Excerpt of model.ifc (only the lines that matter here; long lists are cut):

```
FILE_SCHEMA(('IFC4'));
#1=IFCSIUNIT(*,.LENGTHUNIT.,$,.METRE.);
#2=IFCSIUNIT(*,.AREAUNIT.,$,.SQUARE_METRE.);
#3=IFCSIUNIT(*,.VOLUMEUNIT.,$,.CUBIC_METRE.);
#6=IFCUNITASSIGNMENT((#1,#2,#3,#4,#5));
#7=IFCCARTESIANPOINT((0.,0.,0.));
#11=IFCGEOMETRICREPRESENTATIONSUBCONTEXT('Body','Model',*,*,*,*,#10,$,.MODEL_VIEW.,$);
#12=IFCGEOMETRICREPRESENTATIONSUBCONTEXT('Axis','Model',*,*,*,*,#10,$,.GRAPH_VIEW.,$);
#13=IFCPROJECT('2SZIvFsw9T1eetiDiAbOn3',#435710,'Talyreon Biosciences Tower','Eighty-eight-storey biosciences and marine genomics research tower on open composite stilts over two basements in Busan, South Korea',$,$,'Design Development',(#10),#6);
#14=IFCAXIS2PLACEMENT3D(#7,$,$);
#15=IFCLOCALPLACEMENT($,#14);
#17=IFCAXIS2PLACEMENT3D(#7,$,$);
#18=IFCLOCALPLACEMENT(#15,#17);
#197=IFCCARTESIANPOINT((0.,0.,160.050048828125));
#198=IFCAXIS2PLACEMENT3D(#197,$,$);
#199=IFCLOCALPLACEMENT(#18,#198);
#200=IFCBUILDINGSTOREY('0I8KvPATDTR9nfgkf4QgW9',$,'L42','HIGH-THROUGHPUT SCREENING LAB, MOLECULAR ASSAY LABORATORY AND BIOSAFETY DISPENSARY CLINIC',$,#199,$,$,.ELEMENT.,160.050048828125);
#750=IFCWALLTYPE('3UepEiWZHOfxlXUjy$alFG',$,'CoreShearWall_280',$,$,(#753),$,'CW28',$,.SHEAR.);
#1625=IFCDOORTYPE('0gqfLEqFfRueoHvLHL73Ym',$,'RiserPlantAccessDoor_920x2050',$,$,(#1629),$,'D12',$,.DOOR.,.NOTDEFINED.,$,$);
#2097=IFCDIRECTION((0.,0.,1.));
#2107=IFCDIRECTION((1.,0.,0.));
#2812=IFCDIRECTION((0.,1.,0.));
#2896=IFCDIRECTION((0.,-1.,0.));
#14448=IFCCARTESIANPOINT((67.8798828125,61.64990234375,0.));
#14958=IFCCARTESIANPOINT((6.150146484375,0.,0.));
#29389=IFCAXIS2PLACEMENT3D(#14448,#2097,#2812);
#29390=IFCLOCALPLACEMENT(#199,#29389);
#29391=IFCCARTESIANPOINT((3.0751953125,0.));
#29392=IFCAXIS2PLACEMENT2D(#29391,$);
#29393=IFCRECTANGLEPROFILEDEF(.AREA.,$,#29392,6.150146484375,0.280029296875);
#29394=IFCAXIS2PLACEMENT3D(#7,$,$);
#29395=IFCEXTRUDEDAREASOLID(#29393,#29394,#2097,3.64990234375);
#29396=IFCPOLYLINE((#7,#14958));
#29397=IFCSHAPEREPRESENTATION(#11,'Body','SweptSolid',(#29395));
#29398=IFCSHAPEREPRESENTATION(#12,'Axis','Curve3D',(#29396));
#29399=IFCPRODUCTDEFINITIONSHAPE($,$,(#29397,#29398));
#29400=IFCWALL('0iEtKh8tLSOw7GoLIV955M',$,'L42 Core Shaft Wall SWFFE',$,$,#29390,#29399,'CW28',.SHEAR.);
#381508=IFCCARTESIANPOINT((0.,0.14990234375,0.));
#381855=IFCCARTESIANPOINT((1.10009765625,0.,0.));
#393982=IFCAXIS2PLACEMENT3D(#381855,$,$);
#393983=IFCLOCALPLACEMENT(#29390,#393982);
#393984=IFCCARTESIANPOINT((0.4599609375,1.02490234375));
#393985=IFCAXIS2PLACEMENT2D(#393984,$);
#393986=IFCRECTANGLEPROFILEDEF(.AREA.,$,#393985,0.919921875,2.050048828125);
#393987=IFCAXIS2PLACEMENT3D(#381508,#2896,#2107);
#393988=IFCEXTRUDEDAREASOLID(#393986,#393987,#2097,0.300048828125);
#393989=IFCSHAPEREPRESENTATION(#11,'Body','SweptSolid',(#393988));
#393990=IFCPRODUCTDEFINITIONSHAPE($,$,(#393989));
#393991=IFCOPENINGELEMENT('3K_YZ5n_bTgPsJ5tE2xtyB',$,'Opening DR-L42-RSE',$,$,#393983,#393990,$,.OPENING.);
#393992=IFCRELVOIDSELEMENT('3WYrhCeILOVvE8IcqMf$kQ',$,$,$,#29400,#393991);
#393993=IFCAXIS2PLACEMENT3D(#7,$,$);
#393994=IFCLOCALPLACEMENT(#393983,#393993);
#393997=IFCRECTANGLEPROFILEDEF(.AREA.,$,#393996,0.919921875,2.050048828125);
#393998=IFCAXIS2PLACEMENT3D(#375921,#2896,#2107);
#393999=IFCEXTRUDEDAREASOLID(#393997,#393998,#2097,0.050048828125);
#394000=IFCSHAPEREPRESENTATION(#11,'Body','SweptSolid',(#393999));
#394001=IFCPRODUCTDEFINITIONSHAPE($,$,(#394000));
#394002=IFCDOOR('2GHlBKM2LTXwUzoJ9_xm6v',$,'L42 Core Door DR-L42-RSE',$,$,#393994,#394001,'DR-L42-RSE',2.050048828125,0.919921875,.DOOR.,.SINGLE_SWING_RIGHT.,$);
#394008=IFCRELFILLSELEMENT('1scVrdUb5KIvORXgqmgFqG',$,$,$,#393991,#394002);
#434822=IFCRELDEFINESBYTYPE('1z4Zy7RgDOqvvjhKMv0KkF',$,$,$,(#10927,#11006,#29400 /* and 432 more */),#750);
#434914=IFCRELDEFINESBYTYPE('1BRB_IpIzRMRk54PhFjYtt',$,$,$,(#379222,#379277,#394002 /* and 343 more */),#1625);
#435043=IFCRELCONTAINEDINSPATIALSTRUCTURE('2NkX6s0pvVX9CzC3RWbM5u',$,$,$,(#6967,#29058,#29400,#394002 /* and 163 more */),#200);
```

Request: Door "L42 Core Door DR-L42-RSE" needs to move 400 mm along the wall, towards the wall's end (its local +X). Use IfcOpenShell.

```python
import ifcopenshell
import ifcopenshell.api.geometry
import ifcopenshell.util.placement
import ifcopenshell.util.unit

model = ifcopenshell.open("model.ifc")
unit_scale = ifcopenshell.util.unit.calculate_unit_scale(model)

door = model.by_guid("2GHlBKM2LTXwUzoJ9_xm6v")
opening = door.FillsVoids[0].RelatingOpeningElement
wall = opening.VoidsElements[0].RelatingBuildingElement

wall_matrix = ifcopenshell.util.placement.get_local_placement(wall.ObjectPlacement)
shift = wall_matrix[:3, 0] * 0.4 / unit_scale
before = ifcopenshell.util.placement.get_local_placement(door.ObjectPlacement)[:3, 3].copy()

# The door is placed relative to its opening, so it follows when the opening moves.
matrix = ifcopenshell.util.placement.get_local_placement(opening.ObjectPlacement)
matrix[:3, 3] += shift
ifcopenshell.api.geometry.edit_object_placement(
    model, product=opening, matrix=matrix, is_si=False, should_transform_children=True
)

after = ifcopenshell.util.placement.get_local_placement(door.ObjectPlacement)[:3, 3]
print("door moved by", (after - before).round(3) + 0.0)

model.write("model_v2.ifc")
```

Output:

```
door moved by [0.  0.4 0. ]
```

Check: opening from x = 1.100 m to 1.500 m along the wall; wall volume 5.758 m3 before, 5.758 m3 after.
